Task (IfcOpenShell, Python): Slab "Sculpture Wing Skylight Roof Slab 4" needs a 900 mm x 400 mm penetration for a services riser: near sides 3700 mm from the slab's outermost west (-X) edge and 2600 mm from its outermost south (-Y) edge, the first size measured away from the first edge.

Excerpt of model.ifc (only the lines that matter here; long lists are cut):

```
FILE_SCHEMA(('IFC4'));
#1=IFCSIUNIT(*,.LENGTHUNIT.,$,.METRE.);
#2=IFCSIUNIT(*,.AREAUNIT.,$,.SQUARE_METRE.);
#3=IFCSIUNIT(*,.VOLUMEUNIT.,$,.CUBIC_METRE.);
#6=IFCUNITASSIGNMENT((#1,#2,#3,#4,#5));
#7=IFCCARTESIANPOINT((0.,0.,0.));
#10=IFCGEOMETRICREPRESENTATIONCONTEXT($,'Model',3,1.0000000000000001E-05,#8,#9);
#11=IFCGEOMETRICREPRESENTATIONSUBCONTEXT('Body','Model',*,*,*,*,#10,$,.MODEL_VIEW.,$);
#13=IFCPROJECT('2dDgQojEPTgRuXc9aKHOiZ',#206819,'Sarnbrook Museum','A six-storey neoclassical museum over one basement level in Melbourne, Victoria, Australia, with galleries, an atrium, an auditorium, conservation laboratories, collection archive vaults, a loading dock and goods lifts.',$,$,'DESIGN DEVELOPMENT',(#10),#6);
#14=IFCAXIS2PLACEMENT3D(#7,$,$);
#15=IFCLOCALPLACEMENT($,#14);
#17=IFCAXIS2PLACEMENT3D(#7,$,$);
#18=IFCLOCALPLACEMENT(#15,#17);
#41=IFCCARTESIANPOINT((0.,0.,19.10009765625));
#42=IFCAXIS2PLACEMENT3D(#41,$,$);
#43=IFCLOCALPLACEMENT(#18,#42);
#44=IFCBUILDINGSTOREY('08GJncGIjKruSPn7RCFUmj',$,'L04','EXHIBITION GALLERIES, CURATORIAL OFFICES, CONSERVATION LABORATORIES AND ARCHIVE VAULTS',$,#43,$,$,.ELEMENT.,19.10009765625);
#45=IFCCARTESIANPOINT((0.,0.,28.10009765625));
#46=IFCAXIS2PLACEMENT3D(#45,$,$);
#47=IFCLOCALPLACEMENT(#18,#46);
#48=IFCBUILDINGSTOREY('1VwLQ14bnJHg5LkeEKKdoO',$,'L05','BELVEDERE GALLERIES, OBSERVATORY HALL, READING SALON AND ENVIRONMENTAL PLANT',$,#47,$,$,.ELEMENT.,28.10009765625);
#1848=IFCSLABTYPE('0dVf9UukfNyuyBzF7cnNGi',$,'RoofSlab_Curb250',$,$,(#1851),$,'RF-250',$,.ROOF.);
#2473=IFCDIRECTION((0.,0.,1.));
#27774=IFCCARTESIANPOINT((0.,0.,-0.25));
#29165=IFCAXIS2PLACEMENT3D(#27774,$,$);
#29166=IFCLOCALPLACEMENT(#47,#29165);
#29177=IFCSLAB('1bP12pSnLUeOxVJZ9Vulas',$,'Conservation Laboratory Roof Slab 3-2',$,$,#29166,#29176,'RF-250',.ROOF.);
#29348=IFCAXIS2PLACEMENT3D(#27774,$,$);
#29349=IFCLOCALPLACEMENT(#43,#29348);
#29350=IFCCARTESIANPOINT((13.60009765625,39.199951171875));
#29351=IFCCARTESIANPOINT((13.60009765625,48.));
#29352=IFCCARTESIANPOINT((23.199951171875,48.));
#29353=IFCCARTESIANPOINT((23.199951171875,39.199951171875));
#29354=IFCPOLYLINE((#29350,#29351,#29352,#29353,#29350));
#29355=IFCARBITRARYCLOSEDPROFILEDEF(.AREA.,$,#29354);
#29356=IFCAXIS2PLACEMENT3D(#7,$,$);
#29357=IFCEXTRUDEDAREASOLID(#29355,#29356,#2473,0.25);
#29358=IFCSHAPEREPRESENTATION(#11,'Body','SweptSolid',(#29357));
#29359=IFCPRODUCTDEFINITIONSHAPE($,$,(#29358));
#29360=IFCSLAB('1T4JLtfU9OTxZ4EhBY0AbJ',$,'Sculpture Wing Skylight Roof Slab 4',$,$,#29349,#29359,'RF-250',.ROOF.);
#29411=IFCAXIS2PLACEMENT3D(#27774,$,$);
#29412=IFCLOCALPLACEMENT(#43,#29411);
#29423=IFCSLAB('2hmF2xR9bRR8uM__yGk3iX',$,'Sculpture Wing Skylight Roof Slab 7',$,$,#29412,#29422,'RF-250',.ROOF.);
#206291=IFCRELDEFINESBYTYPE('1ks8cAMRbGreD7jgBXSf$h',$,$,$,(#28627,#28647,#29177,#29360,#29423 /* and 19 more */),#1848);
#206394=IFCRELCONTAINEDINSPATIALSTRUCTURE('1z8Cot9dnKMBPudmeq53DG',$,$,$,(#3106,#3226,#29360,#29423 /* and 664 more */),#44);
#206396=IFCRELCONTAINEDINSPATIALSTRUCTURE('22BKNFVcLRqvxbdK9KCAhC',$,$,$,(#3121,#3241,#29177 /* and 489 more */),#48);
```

```python
import numpy as np
import ifcopenshell
import ifcopenshell.api.feature
import ifcopenshell.api.geometry
import ifcopenshell.api.root
import ifcopenshell.geom
import ifcopenshell.util.placement
import ifcopenshell.util.representation
import ifcopenshell.util.shape
import ifcopenshell.util.unit

model = ifcopenshell.open("model.ifc")
unit_scale = ifcopenshell.util.unit.calculate_unit_scale(model)
settings = ifcopenshell.geom.settings()


def volume(element):
    """Net volume in cubic metres, openings subtracted."""
    shape = ifcopenshell.geom.create_shape(settings, element)
    return ifcopenshell.util.shape.get_volume(shape.geometry)


slab = model.by_id(29360)
before = volume(slab)

# Extent in the slab's own axes, in metres. The edges named are its -X and -Y sides.
slab_shape = ifcopenshell.geom.create_shape(settings, slab)
vertices = ifcopenshell.util.shape.get_vertices(slab_shape.geometry)
x_min, y_min, bottom = vertices.min(axis=0)
top = vertices[:, 2].max()

opening = ifcopenshell.api.root.create_entity(model, ifc_class="IfcOpeningElement", name="Services riser opening", predefined_type="OPENING")
context = ifcopenshell.util.representation.get_context(model, "Model", "Body", "MODEL_VIEW")
width, depth = 0.9, 0.4
outline = [(0.0, 0.0), (width, 0.0), (width, depth), (0.0, depth), (0.0, 0.0)]
# Overshoot both faces by 50 mm so the cut is clean.
shape = ifcopenshell.api.geometry.add_slab_representation(
    model, context=context, depth=top - bottom + 0.1, polyline=outline
)
ifcopenshell.api.geometry.assign_representation(model, product=opening, representation=shape)

matrix = ifcopenshell.util.placement.get_local_placement(slab.ObjectPlacement)
matrix[:, 3] = matrix @ np.append(np.array([x_min + 3.7, y_min + 2.6, bottom - 0.05]) / unit_scale, 1.0)
ifcopenshell.api.geometry.edit_object_placement(model, product=opening, matrix=matrix, is_si=False)
ifcopenshell.api.feature.add_feature(model, feature=opening, element=slab)

after = volume(slab)

print(f"slab volume {before:.3f} -> {after:.3f} m3")

model.write("model_rev.ifc")
```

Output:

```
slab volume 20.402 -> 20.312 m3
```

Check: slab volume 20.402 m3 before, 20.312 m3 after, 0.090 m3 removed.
